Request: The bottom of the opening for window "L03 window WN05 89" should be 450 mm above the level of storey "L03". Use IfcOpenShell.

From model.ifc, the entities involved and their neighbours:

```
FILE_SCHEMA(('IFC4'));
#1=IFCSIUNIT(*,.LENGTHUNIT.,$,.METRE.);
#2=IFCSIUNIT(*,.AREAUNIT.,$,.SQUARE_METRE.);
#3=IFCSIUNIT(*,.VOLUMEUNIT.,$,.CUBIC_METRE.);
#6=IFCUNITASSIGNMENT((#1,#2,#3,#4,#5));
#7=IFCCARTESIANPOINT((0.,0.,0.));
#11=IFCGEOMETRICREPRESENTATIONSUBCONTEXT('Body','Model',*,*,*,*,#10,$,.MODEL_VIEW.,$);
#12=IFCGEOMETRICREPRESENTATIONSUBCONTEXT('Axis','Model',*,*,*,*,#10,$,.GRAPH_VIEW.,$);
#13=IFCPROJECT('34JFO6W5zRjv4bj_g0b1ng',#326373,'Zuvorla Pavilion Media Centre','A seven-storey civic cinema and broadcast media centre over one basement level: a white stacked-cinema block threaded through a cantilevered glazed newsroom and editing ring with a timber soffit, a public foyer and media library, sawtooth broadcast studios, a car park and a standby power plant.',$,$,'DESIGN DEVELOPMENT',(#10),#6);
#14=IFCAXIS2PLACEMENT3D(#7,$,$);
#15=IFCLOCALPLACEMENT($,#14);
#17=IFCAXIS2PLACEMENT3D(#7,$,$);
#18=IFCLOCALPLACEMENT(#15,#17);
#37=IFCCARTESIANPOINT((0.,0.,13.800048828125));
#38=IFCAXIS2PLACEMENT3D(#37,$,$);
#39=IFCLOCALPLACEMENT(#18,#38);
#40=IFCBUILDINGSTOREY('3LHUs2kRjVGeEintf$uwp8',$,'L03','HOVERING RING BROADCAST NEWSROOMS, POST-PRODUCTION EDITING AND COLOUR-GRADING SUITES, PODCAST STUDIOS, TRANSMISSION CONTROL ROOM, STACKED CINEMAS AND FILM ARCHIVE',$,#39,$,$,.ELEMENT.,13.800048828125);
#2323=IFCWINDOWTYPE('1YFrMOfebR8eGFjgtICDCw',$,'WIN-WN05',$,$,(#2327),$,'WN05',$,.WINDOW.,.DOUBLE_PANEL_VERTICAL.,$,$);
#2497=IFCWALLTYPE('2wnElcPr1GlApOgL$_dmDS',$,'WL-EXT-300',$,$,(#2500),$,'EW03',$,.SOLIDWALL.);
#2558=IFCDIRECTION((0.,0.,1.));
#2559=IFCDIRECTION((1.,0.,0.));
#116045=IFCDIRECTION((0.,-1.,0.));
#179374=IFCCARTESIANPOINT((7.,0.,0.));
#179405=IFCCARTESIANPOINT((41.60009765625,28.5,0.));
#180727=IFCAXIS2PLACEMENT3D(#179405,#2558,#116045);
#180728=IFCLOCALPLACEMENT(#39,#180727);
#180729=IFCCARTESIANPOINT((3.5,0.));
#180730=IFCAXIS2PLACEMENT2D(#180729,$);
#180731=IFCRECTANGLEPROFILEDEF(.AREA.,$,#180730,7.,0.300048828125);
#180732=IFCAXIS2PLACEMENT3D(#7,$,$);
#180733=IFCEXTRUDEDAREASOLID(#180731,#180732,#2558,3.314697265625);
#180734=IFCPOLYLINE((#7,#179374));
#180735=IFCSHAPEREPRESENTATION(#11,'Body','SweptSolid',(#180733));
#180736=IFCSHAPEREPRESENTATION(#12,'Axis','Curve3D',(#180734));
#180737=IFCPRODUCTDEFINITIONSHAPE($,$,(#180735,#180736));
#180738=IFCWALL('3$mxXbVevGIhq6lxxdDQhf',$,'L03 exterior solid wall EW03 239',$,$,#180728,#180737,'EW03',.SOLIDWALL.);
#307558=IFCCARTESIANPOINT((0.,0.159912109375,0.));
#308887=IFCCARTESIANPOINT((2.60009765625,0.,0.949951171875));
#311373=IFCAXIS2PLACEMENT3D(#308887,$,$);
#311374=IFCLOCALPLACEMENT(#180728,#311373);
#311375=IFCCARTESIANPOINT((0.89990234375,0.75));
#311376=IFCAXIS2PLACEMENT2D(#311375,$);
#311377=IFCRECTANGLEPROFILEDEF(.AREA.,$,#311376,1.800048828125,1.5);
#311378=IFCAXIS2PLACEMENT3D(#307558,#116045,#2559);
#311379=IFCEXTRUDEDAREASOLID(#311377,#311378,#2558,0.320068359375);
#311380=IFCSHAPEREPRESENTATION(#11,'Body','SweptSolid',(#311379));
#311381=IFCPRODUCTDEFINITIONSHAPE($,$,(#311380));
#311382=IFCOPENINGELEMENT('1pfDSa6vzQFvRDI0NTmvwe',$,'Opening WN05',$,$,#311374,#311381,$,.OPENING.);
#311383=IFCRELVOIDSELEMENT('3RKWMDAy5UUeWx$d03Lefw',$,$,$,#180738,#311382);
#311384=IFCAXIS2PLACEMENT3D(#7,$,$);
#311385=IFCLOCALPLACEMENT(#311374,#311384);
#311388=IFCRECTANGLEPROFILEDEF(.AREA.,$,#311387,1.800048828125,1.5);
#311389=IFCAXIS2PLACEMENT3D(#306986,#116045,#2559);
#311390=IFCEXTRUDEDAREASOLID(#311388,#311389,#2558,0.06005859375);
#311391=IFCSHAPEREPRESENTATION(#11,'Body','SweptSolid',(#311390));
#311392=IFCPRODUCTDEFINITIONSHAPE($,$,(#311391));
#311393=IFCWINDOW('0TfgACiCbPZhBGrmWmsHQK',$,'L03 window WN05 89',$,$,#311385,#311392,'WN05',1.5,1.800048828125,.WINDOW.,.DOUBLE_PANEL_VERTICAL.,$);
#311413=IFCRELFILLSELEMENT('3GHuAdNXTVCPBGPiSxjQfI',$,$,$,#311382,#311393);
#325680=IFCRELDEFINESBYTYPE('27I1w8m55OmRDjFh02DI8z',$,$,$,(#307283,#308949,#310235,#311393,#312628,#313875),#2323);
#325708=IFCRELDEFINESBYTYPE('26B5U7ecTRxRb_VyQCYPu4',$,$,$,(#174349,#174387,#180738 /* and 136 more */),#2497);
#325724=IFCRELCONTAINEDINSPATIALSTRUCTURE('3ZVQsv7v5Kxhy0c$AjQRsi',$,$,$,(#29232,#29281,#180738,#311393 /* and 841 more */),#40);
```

```python
import numpy as np
import ifcopenshell
import ifcopenshell.api.geometry
import ifcopenshell.geom
import ifcopenshell.util.element
import ifcopenshell.util.placement
import ifcopenshell.util.shape
import ifcopenshell.util.unit

model = ifcopenshell.open("model.ifc")
unit_scale = ifcopenshell.util.unit.calculate_unit_scale(model)

window = model.by_guid("0TfgACiCbPZhBGrmWmsHQK")
opening = window.FillsVoids[0].RelatingOpeningElement
storey = ifcopenshell.util.element.get_container(window, ifc_class="IfcBuildingStorey")
level = ifcopenshell.util.placement.get_local_placement(storey.ObjectPlacement)[2, 3]

# The opening's origin need not be at the sill, so measure its lowest point.
shape = ifcopenshell.geom.create_shape(ifcopenshell.geom.settings(), opening)
bottom = ifcopenshell.util.shape.get_shape_bottom_elevation(shape, shape.geometry) / unit_scale
dz = level + 0.45 / unit_scale - bottom

shift = np.array([0.0, 0.0, dz])
# The window is placed relative to its opening, so it follows when the opening moves.
matrix = ifcopenshell.util.placement.get_local_placement(opening.ObjectPlacement)
matrix[:3, 3] += shift
ifcopenshell.api.geometry.edit_object_placement(
    model, product=opening, matrix=matrix, is_si=False, should_transform_children=True
)

print(f"moved by {dz * unit_scale:+.3f} m")

model.write("model_v2.ifc")
```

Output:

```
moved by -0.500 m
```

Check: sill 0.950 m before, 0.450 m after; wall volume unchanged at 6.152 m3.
